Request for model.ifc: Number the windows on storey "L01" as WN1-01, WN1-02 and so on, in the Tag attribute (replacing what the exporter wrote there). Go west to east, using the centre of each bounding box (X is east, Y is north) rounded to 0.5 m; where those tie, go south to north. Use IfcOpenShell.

First a look at what the model holds.

```python
import ifcopenshell
import ifcopenshell.util.element
import ifcopenshell.util.placement

model = ifcopenshell.open("model.ifc")
print(model.schema)
storey = next(s for s in model.by_type("IfcBuildingStorey") if s.Name == "L01")
windows = [e for e in ifcopenshell.util.element.get_decomposition(storey) if e.is_a("IfcWindow")]
for e in sorted(windows, key=lambda e: e.id()):
    origin = ifcopenshell.util.placement.get_local_placement(e.ObjectPlacement)[:3, 3]
    print(e.id(), e.Tag, e.Name, origin.round(2) + 0.0, sep=" | ")
```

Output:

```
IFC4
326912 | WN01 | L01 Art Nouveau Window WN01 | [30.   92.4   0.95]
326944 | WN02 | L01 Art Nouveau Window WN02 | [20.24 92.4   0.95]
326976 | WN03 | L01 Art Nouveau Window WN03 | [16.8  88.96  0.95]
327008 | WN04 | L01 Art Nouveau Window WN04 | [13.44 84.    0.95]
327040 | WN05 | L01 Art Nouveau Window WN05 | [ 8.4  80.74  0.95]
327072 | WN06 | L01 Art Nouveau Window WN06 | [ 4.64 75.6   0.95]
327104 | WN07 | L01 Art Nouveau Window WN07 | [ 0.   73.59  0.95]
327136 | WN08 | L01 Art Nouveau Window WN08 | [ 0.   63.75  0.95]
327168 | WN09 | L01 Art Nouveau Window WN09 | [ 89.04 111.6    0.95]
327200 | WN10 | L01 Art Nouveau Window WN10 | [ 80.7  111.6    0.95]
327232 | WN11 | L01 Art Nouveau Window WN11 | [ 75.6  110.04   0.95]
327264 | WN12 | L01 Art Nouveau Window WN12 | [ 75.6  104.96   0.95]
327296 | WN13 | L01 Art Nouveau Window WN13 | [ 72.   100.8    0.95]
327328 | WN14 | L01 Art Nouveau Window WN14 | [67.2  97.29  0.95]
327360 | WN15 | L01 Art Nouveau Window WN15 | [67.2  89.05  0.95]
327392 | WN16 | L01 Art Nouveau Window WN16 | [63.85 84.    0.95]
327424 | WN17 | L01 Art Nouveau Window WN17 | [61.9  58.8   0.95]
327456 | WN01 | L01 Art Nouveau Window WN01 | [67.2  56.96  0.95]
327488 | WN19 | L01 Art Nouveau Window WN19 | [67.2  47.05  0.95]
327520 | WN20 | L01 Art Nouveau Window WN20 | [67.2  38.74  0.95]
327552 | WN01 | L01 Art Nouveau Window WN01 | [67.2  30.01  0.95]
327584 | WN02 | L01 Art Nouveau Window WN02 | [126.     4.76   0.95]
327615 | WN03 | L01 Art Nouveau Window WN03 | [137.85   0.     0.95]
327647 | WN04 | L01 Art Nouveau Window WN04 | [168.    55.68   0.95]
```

```python
import ifcopenshell
import ifcopenshell.geom
import ifcopenshell.util.element
import ifcopenshell.util.shape

model = ifcopenshell.open("model.ifc")
settings = ifcopenshell.geom.settings()
settings.set("use-world-coords", True)


def centre(element):
    shape = ifcopenshell.geom.create_shape(settings, element)
    return ifcopenshell.util.shape.get_bbox_centroid(shape.geometry)


storey = next(s for s in model.by_type("IfcBuildingStorey") if s.Name == "L01")
windows = [e for e in ifcopenshell.util.element.get_decomposition(storey) if e.is_a("IfcWindow")]

# Insertion points can sit at a corner or the storey origin, so sort by the geometry (in metres).
centres = {e: centre(e) for e in windows}
windows.sort(key=lambda e: (round(centres[e][0] / 0.5), centres[e][1]))

for i, e in enumerate(windows, start=1):
    number = f"WN1-{i:02d}"
    e.Tag = number
    print(e.id(), number)

model.write("model_rev.ifc")
```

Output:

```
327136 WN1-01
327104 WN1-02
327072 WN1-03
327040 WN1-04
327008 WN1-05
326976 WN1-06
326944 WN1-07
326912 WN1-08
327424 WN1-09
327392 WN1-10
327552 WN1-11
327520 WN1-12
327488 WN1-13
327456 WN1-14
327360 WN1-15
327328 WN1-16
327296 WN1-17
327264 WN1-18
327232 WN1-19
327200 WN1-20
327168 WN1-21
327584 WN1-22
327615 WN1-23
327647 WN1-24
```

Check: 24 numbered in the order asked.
